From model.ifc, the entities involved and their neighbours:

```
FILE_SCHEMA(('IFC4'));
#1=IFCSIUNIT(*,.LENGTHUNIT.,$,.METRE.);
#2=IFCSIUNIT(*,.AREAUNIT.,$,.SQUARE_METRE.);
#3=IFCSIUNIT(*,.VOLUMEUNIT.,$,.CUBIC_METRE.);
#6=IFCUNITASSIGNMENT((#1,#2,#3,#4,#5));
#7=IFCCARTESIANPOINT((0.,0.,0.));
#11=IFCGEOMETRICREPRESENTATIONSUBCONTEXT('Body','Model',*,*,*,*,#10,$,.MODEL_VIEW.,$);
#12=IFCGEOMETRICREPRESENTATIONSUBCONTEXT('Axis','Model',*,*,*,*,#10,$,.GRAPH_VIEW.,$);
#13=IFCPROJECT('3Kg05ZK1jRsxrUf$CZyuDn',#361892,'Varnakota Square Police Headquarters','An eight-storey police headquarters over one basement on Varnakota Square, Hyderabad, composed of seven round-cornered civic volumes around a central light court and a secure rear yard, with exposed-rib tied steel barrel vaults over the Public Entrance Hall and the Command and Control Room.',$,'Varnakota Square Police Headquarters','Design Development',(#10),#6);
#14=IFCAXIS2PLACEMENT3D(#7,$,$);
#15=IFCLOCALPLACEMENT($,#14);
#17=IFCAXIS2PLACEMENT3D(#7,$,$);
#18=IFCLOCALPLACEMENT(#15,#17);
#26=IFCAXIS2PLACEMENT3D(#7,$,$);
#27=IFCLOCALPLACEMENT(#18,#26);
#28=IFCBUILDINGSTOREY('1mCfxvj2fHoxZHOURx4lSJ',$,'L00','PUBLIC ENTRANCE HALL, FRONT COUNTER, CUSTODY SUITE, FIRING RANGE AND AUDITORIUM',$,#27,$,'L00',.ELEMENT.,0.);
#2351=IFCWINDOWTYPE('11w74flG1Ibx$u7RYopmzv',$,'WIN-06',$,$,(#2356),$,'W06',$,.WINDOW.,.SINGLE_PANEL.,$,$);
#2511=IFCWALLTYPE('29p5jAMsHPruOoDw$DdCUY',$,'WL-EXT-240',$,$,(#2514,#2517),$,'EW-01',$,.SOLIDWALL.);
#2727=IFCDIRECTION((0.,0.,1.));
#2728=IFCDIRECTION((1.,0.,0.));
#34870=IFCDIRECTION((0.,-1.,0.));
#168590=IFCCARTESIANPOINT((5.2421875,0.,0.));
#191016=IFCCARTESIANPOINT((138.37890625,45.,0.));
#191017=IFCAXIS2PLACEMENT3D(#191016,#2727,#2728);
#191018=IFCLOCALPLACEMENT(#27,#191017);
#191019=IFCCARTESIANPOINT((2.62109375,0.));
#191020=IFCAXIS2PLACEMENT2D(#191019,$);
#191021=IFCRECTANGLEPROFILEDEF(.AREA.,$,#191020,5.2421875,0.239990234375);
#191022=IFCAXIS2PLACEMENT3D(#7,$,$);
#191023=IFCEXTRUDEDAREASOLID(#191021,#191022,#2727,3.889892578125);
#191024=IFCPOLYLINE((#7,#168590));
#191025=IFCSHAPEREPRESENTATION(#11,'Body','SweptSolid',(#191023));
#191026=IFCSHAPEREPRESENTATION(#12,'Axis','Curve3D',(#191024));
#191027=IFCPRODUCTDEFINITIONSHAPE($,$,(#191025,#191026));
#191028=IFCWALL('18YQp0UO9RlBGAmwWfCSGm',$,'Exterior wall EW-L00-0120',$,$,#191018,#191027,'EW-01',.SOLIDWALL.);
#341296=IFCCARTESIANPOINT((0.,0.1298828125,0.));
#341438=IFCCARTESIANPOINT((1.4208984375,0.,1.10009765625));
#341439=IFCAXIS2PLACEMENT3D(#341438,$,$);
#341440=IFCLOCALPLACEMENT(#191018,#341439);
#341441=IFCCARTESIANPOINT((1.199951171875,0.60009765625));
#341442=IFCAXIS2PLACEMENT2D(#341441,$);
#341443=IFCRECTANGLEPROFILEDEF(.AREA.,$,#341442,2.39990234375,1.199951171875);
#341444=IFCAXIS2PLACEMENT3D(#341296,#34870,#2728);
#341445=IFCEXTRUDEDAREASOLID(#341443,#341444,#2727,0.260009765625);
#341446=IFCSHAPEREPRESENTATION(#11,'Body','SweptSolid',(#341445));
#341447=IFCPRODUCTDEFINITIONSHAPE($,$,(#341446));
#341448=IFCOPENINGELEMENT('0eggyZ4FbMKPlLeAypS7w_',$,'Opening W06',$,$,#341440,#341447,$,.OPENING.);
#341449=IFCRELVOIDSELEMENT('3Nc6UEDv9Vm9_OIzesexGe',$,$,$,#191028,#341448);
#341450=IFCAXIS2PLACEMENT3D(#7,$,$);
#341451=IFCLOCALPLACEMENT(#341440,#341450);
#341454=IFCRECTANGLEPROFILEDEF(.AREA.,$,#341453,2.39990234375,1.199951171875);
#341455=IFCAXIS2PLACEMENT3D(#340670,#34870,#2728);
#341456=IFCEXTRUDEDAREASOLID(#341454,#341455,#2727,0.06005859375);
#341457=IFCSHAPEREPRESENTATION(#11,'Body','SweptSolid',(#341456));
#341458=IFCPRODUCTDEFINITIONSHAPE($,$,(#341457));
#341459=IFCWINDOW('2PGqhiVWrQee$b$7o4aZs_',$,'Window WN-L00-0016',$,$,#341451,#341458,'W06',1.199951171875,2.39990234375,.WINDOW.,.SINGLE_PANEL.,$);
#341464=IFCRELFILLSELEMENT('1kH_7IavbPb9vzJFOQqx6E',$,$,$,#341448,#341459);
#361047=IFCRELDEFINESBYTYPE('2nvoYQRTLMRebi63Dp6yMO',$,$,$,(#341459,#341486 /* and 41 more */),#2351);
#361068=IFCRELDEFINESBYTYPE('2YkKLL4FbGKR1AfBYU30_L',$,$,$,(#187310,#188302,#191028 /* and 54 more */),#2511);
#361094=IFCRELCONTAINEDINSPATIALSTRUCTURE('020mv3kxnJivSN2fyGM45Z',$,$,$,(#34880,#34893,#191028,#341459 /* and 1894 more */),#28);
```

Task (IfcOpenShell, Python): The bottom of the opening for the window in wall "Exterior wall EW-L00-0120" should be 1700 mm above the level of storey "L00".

```python
import numpy as np
import ifcopenshell
import ifcopenshell.api.geometry
import ifcopenshell.geom
import ifcopenshell.util.element
import ifcopenshell.util.placement
import ifcopenshell.util.shape
import ifcopenshell.util.unit

model = ifcopenshell.open("model.ifc")
unit_scale = ifcopenshell.util.unit.calculate_unit_scale(model)

window = model.by_guid("2PGqhiVWrQee$b$7o4aZs_")
opening = window.FillsVoids[0].RelatingOpeningElement
storey = ifcopenshell.util.element.get_container(window, ifc_class="IfcBuildingStorey")
level = ifcopenshell.util.placement.get_local_placement(storey.ObjectPlacement)[2, 3]

# The opening's origin need not be at the sill, so measure its lowest point.
shape = ifcopenshell.geom.create_shape(ifcopenshell.geom.settings(), opening)
bottom = ifcopenshell.util.shape.get_shape_bottom_elevation(shape, shape.geometry) / unit_scale
dz = level + 1.7 / unit_scale - bottom

shift = np.array([0.0, 0.0, dz])
# The window is placed relative to its opening, so it follows when the opening moves.
matrix = ifcopenshell.util.placement.get_local_placement(opening.ObjectPlacement)
matrix[:3, 3] += shift
ifcopenshell.api.geometry.edit_object_placement(
    model, product=opening, matrix=matrix, is_si=False, should_transform_children=True
)

print(f"moved by {dz * unit_scale:+.3f} m")

model.write("model_rev.ifc")
```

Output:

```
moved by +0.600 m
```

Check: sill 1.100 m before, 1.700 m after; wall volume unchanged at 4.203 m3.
